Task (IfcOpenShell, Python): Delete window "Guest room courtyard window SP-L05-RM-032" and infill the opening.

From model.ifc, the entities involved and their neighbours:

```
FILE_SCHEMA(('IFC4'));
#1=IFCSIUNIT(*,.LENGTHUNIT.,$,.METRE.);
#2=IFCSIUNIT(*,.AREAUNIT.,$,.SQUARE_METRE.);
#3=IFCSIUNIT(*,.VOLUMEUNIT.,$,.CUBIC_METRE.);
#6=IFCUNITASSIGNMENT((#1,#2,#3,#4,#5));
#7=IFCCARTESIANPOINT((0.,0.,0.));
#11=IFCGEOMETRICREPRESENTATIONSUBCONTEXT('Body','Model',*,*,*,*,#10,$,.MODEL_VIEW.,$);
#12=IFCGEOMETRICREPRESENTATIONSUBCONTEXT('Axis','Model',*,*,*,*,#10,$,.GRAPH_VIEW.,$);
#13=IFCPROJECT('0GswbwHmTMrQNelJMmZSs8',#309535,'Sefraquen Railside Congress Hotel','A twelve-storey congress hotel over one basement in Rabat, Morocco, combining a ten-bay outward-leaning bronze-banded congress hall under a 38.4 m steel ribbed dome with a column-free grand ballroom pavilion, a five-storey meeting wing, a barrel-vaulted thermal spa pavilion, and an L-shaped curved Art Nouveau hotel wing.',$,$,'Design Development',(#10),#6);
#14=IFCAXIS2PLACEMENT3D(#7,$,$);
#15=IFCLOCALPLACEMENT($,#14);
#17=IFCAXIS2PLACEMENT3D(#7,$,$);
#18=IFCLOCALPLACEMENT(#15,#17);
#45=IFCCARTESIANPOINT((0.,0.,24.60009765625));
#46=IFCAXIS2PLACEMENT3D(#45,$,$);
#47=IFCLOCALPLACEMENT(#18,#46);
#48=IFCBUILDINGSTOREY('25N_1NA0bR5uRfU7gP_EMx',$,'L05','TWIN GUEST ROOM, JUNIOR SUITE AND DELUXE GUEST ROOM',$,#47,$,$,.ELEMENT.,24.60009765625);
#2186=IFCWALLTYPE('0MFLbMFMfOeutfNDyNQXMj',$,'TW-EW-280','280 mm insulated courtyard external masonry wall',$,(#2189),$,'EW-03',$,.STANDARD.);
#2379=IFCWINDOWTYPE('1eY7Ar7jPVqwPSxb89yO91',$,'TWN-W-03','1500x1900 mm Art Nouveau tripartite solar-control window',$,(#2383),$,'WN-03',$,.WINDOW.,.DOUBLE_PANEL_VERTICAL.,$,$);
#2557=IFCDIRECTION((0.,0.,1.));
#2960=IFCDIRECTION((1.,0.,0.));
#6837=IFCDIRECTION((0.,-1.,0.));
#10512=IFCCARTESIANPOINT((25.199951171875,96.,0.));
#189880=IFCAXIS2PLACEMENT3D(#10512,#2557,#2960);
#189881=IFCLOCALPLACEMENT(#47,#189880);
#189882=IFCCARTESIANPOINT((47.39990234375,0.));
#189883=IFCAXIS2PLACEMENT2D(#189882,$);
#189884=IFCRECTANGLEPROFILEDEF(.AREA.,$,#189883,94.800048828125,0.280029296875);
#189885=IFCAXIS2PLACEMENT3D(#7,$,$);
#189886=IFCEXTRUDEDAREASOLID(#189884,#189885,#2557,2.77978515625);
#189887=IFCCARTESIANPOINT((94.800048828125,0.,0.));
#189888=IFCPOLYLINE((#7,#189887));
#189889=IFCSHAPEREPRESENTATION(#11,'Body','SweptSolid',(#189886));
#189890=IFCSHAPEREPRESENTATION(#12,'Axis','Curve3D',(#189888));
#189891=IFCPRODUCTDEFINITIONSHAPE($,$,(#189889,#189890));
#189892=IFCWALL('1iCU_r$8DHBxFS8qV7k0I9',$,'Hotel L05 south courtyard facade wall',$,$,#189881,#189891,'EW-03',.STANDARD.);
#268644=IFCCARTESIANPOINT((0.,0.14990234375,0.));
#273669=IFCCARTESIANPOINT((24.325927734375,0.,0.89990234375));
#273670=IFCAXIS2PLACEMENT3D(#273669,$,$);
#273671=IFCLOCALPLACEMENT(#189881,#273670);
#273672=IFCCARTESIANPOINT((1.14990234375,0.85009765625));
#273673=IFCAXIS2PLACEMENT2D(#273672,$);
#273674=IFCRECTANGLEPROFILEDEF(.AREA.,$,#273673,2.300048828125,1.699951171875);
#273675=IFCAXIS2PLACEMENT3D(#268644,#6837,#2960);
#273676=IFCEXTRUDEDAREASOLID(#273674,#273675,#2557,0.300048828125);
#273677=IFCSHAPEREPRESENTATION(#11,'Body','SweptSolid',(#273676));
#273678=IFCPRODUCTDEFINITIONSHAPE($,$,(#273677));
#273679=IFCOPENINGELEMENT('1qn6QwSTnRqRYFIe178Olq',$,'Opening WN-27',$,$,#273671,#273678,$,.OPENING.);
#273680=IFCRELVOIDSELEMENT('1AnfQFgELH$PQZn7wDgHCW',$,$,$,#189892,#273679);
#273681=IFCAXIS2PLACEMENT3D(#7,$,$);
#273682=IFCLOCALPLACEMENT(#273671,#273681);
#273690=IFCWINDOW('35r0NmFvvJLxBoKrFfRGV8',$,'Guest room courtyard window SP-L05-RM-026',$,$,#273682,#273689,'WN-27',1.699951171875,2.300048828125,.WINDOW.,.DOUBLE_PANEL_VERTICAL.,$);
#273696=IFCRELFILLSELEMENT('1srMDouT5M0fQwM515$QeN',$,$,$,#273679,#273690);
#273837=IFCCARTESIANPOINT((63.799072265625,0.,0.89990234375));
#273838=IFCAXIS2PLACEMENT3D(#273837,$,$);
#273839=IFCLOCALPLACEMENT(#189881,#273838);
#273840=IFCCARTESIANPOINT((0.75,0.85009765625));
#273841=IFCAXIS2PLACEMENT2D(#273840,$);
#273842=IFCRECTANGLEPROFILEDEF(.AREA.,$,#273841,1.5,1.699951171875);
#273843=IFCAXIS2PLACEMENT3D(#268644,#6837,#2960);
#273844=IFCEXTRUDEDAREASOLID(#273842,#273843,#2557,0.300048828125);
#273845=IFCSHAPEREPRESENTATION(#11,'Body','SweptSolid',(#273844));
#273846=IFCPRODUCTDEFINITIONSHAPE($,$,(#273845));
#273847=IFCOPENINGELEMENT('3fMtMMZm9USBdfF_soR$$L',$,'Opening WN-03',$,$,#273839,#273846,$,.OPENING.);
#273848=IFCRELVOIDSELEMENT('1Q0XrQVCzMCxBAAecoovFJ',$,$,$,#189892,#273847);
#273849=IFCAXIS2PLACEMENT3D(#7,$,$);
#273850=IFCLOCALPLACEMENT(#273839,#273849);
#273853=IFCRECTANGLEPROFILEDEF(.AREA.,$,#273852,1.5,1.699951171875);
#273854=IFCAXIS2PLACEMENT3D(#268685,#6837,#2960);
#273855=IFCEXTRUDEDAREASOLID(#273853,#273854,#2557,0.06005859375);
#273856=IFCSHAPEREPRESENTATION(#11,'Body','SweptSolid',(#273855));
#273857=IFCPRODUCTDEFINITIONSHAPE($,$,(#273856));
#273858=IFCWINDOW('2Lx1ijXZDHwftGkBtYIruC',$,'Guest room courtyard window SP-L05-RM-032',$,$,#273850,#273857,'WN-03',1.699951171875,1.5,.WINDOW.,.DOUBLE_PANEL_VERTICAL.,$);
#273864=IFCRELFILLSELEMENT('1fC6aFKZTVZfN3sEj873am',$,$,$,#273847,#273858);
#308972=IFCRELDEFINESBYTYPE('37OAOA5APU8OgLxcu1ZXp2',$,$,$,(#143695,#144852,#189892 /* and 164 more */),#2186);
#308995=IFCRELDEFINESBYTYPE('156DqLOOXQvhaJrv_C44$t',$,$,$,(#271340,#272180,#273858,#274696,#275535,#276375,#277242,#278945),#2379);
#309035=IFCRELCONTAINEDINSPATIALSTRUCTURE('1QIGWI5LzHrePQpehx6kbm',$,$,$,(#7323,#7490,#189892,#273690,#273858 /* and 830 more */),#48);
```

```python
import ifcopenshell
import ifcopenshell.api.feature
import ifcopenshell.api.root
import ifcopenshell.geom
import ifcopenshell.util.shape

model = ifcopenshell.open("model.ifc")
settings = ifcopenshell.geom.settings()


def volume(element):
    """Net volume in cubic metres, openings subtracted."""
    shape = ifcopenshell.geom.create_shape(settings, element)
    return ifcopenshell.util.shape.get_volume(shape.geometry)


window = model.by_id(273858)
opening = window.FillsVoids[0].RelatingOpeningElement
wall = opening.VoidsElements[0].RelatingBuildingElement
before = volume(wall)

ifcopenshell.api.root.remove_product(model, product=window)
ifcopenshell.api.feature.remove_feature(model, feature=opening)

after = volume(wall)

print(f"wall volume {before:.3f} -> {after:.3f} m3")

model.write("model_edited.ifc")
```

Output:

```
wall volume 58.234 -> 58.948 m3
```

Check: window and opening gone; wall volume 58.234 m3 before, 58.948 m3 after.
